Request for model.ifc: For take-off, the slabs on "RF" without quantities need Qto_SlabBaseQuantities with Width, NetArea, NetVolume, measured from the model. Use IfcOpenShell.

First a look at what the model holds.

```python
import ifcopenshell
import ifcopenshell.util.element
import ifcopenshell.util.unit

model = ifcopenshell.open("model.ifc")
print(model.schema)
for unit_type in ("LENGTHUNIT", "AREAUNIT", "VOLUMEUNIT"):
    print(unit_type, ifcopenshell.util.unit.calculate_unit_scale(model, unit_type))
storey = next(s for s in model.by_type("IfcBuildingStorey") if s.Name == "RF")
slabs = [e for e in ifcopenshell.util.element.get_decomposition(storey) if e.is_a("IfcSlab")]
for e in sorted(slabs, key=lambda e: e.id()):
    print(e.id(), e.is_a(), e.Name, list(ifcopenshell.util.element.get_psets(e, qtos_only=True)), sep=" | ")
```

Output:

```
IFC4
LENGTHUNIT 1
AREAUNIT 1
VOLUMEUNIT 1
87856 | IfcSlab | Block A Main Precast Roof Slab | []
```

```python
import ifcopenshell
import ifcopenshell.api.pset
import ifcopenshell.geom
import ifcopenshell.util.element
import ifcopenshell.util.shape
import ifcopenshell.util.unit

model = ifcopenshell.open("model.ifc")
unit_scale = ifcopenshell.util.unit.calculate_unit_scale(model)
area_scale = ifcopenshell.util.unit.calculate_unit_scale(model, "AREAUNIT")
volume_scale = ifcopenshell.util.unit.calculate_unit_scale(model, "VOLUMEUNIT")
settings = ifcopenshell.geom.settings()

storey = next(s for s in model.by_type("IfcBuildingStorey") if s.Name == "RF")
slabs = [e for e in ifcopenshell.util.element.get_decomposition(storey) if e.is_a("IfcSlab")]

for e in sorted(slabs, key=lambda e: e.id()):
    if ifcopenshell.util.element.get_psets(e, qtos_only=True, should_inherit=False):
        continue
    # Geometry comes back in metres, in the element's own axes.
    shape = ifcopenshell.geom.create_shape(settings, e)
    values = {
        "Width": ifcopenshell.util.shape.get_z(shape.geometry) / unit_scale,
        "NetArea": ifcopenshell.util.shape.get_footprint_area(shape.geometry) / area_scale,
        "NetVolume": ifcopenshell.util.shape.get_volume(shape.geometry) / volume_scale,
    }
    qto = ifcopenshell.api.pset.add_qto(model, product=e, name="Qto_SlabBaseQuantities")
    ifcopenshell.api.pset.edit_qto(model, qto=qto, properties=values)
    print(e.id(), {k: round(v, 3) for k, v in values.items()})

model.write("model_v2.ifc")
```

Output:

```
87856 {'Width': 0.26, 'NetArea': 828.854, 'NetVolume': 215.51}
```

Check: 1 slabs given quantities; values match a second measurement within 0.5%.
